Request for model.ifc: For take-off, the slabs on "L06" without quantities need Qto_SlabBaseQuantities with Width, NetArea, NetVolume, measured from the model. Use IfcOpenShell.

First a look at what the model holds.

```python
import ifcopenshell
import ifcopenshell.util.element
import ifcopenshell.util.unit

model = ifcopenshell.open("model.ifc")
print(model.schema)
for unit_type in ("LENGTHUNIT", "AREAUNIT", "VOLUMEUNIT"):
    print(unit_type, ifcopenshell.util.unit.calculate_unit_scale(model, unit_type))
storey = next(s for s in model.by_type("IfcBuildingStorey") if s.Name == "L06")
slabs = [e for e in ifcopenshell.util.element.get_decomposition(storey) if e.is_a("IfcSlab")]
for e in sorted(slabs, key=lambda e: e.id()):
    print(e.id(), e.is_a(), e.Name, list(ifcopenshell.util.element.get_psets(e, qtos_only=True)), sep=" | ")
```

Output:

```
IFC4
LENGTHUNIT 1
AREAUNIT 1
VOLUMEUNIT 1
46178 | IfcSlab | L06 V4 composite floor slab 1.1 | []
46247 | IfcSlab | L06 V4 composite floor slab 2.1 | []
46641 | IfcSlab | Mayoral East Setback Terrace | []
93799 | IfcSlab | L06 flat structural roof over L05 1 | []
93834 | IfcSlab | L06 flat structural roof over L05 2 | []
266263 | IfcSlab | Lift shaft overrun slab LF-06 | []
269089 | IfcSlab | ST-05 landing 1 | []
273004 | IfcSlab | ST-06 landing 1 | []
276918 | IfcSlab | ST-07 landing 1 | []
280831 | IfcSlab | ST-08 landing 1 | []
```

```python
import ifcopenshell
import ifcopenshell.api.pset
import ifcopenshell.geom
import ifcopenshell.util.element
import ifcopenshell.util.shape
import ifcopenshell.util.unit

model = ifcopenshell.open("model.ifc")
unit_scale = ifcopenshell.util.unit.calculate_unit_scale(model)
area_scale = ifcopenshell.util.unit.calculate_unit_scale(model, "AREAUNIT")
volume_scale = ifcopenshell.util.unit.calculate_unit_scale(model, "VOLUMEUNIT")
settings = ifcopenshell.geom.settings()

storey = next(s for s in model.by_type("IfcBuildingStorey") if s.Name == "L06")
slabs = [e for e in ifcopenshell.util.element.get_decomposition(storey) if e.is_a("IfcSlab")]

for e in sorted(slabs, key=lambda e: e.id()):
    if ifcopenshell.util.element.get_psets(e, qtos_only=True, should_inherit=False):
        continue
    # Geometry comes back in metres, in the element's own axes.
    shape = ifcopenshell.geom.create_shape(settings, e)
    values = {
        "Width": ifcopenshell.util.shape.get_z(shape.geometry) / unit_scale,
        "NetArea": ifcopenshell.util.shape.get_footprint_area(shape.geometry) / area_scale,
        "NetVolume": ifcopenshell.util.shape.get_volume(shape.geometry) / volume_scale,
    }
    qto = ifcopenshell.api.pset.add_qto(model, product=e, name="Qto_SlabBaseQuantities")
    ifcopenshell.api.pset.edit_qto(model, qto=qto, properties=values)
    print(e.id(), {k: round(v, 3) for k, v in values.items()})

model.write("model-out.ifc")
```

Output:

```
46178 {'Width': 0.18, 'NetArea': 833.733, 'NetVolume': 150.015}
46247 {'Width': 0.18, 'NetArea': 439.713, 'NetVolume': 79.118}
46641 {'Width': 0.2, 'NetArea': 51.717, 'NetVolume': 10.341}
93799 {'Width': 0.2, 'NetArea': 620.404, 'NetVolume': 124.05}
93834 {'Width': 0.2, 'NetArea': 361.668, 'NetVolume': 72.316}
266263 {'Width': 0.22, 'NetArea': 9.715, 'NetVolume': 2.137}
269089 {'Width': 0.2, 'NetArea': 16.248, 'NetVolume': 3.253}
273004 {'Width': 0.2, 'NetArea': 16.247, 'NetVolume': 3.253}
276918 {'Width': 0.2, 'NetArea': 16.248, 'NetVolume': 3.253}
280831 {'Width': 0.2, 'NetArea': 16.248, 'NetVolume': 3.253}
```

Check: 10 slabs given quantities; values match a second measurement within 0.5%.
